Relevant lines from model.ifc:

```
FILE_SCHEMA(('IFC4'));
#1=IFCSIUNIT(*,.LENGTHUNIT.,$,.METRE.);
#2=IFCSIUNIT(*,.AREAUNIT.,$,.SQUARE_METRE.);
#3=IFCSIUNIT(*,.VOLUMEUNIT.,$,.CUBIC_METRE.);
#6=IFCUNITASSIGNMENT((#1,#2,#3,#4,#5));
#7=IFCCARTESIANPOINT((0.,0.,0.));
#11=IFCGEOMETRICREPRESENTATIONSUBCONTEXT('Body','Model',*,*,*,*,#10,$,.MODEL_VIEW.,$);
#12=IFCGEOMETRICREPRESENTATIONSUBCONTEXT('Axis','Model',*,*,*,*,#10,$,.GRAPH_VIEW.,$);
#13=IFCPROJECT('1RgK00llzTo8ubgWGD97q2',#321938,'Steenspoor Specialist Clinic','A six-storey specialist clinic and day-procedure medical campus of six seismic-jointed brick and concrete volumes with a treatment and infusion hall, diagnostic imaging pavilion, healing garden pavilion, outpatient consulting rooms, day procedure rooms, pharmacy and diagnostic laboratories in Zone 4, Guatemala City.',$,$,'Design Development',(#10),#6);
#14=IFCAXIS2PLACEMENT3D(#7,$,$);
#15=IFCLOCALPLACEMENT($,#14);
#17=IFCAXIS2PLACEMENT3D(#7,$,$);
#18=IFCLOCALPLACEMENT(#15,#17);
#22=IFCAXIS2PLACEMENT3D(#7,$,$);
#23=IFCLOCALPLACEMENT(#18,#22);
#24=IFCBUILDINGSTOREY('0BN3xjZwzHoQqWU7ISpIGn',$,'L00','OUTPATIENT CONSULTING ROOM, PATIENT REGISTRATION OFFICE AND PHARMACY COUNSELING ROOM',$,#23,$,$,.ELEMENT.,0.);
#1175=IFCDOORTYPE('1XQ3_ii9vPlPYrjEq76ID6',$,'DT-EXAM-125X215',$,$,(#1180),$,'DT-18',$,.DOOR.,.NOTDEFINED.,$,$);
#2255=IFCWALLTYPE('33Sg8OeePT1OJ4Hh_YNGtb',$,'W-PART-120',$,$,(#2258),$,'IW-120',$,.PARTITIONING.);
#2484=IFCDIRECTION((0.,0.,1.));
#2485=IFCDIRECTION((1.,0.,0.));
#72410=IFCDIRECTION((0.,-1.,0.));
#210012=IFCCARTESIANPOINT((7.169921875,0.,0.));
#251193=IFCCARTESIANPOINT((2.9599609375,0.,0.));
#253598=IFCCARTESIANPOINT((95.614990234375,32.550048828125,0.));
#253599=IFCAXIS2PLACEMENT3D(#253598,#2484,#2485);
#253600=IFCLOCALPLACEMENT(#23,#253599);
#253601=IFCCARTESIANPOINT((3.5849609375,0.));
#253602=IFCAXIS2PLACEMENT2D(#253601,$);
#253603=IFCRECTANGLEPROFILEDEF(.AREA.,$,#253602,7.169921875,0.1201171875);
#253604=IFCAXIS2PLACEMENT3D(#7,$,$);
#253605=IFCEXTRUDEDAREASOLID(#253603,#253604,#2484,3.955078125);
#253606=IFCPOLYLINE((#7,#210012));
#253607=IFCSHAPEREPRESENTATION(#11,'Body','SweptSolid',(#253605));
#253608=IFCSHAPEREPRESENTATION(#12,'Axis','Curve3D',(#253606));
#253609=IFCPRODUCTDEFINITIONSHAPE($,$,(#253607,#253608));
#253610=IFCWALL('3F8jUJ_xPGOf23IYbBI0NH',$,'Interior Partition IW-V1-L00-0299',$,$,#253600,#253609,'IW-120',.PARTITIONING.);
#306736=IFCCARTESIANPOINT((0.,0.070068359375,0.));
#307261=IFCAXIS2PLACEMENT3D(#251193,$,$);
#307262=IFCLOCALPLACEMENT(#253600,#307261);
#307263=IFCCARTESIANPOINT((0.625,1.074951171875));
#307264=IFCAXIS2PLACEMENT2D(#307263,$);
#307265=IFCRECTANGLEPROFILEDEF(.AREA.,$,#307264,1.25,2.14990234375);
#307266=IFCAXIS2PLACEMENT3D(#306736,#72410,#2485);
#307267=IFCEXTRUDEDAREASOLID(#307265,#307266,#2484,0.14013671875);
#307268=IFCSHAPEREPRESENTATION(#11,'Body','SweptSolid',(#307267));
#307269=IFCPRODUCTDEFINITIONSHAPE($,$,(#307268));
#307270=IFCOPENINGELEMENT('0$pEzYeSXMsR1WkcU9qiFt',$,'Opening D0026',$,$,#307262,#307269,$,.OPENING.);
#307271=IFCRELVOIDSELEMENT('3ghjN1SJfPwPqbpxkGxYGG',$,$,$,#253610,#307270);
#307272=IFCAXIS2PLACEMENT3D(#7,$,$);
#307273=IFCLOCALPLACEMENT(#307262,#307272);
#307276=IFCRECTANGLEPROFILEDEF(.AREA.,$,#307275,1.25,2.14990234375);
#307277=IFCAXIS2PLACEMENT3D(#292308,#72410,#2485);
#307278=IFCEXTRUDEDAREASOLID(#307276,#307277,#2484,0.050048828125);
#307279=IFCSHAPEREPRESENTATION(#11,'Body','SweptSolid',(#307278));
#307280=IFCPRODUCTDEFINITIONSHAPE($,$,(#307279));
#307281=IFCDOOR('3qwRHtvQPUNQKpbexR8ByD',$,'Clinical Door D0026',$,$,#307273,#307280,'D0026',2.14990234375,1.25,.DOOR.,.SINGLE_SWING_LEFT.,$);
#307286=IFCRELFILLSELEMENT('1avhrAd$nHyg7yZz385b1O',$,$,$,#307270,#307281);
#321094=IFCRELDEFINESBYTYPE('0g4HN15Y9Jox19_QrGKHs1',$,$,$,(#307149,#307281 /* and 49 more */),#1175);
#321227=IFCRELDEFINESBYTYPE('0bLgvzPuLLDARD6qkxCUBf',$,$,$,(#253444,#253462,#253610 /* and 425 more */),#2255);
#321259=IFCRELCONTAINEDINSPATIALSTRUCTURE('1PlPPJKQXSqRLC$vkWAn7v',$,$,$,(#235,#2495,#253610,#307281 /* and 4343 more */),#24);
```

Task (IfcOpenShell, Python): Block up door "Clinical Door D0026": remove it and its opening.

```python
import ifcopenshell
import ifcopenshell.api.feature
import ifcopenshell.api.root
import ifcopenshell.geom
import ifcopenshell.util.shape

model = ifcopenshell.open("model.ifc")
settings = ifcopenshell.geom.settings()


def volume(element):
    """Net volume in cubic metres, openings subtracted."""
    shape = ifcopenshell.geom.create_shape(settings, element)
    return ifcopenshell.util.shape.get_volume(shape.geometry)


door = model.by_guid("3qwRHtvQPUNQKpbexR8ByD")
opening = door.FillsVoids[0].RelatingOpeningElement
wall = opening.VoidsElements[0].RelatingBuildingElement
before = volume(wall)

ifcopenshell.api.root.remove_product(model, product=door)
ifcopenshell.api.feature.remove_feature(model, feature=opening)

after = volume(wall)

print(f"wall volume {before:.3f} -> {after:.3f} m3")

model.write("model-out.ifc")
```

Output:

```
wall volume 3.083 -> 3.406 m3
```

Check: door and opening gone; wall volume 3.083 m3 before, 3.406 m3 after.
